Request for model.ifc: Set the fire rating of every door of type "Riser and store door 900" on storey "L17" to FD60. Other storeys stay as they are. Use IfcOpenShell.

First a look at what the model holds.

```python
import ifcopenshell
import ifcopenshell.util.element

model = ifcopenshell.open("model.ifc")
print(model.schema)
storey = next(s for s in model.by_type("IfcBuildingStorey") if s.Name == "L17")
doors = [e for e in ifcopenshell.util.element.get_decomposition(storey) if e.is_a("IfcDoor")]
seen = {}
for e in doors:
    element_type = ifcopenshell.util.element.get_type(e)
    key = (element_type.Name if element_type != e and element_type else None, ifcopenshell.util.element.get_pset(e, "Pset_DoorCommon", "FireRating"))
    seen[key] = seen.get(key, 0) + 1
for (name, value), count in sorted(seen.items(), key=str):
    print(count, "x", name, "|", value)
```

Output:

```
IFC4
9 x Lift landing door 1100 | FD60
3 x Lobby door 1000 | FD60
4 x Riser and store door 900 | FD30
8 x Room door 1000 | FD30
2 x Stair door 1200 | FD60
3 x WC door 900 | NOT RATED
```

```python
import ifcopenshell
import ifcopenshell.api.pset
import ifcopenshell.util.element

model = ifcopenshell.open("model.ifc")

storey = next(s for s in model.by_type("IfcBuildingStorey") if s.Name == "L17")
doors = [e for e in ifcopenshell.util.element.get_decomposition(storey) if e.is_a("IfcDoor")]

count = 0
for e in doors:
    element_type = ifcopenshell.util.element.get_type(e)
    if element_type in (None, e) or element_type.Name != "Riser and store door 900":
        continue
    # add_pset returns the element's existing set when there is one.
    pset = ifcopenshell.api.pset.add_pset(model, product=e, name="Pset_DoorCommon")
    ifcopenshell.api.pset.edit_pset(model, pset=pset, properties={"FireRating": "FD60"})
    count += 1

print(count, "doors updated")

model.write("model_v2.ifc")
```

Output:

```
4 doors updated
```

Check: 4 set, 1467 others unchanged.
